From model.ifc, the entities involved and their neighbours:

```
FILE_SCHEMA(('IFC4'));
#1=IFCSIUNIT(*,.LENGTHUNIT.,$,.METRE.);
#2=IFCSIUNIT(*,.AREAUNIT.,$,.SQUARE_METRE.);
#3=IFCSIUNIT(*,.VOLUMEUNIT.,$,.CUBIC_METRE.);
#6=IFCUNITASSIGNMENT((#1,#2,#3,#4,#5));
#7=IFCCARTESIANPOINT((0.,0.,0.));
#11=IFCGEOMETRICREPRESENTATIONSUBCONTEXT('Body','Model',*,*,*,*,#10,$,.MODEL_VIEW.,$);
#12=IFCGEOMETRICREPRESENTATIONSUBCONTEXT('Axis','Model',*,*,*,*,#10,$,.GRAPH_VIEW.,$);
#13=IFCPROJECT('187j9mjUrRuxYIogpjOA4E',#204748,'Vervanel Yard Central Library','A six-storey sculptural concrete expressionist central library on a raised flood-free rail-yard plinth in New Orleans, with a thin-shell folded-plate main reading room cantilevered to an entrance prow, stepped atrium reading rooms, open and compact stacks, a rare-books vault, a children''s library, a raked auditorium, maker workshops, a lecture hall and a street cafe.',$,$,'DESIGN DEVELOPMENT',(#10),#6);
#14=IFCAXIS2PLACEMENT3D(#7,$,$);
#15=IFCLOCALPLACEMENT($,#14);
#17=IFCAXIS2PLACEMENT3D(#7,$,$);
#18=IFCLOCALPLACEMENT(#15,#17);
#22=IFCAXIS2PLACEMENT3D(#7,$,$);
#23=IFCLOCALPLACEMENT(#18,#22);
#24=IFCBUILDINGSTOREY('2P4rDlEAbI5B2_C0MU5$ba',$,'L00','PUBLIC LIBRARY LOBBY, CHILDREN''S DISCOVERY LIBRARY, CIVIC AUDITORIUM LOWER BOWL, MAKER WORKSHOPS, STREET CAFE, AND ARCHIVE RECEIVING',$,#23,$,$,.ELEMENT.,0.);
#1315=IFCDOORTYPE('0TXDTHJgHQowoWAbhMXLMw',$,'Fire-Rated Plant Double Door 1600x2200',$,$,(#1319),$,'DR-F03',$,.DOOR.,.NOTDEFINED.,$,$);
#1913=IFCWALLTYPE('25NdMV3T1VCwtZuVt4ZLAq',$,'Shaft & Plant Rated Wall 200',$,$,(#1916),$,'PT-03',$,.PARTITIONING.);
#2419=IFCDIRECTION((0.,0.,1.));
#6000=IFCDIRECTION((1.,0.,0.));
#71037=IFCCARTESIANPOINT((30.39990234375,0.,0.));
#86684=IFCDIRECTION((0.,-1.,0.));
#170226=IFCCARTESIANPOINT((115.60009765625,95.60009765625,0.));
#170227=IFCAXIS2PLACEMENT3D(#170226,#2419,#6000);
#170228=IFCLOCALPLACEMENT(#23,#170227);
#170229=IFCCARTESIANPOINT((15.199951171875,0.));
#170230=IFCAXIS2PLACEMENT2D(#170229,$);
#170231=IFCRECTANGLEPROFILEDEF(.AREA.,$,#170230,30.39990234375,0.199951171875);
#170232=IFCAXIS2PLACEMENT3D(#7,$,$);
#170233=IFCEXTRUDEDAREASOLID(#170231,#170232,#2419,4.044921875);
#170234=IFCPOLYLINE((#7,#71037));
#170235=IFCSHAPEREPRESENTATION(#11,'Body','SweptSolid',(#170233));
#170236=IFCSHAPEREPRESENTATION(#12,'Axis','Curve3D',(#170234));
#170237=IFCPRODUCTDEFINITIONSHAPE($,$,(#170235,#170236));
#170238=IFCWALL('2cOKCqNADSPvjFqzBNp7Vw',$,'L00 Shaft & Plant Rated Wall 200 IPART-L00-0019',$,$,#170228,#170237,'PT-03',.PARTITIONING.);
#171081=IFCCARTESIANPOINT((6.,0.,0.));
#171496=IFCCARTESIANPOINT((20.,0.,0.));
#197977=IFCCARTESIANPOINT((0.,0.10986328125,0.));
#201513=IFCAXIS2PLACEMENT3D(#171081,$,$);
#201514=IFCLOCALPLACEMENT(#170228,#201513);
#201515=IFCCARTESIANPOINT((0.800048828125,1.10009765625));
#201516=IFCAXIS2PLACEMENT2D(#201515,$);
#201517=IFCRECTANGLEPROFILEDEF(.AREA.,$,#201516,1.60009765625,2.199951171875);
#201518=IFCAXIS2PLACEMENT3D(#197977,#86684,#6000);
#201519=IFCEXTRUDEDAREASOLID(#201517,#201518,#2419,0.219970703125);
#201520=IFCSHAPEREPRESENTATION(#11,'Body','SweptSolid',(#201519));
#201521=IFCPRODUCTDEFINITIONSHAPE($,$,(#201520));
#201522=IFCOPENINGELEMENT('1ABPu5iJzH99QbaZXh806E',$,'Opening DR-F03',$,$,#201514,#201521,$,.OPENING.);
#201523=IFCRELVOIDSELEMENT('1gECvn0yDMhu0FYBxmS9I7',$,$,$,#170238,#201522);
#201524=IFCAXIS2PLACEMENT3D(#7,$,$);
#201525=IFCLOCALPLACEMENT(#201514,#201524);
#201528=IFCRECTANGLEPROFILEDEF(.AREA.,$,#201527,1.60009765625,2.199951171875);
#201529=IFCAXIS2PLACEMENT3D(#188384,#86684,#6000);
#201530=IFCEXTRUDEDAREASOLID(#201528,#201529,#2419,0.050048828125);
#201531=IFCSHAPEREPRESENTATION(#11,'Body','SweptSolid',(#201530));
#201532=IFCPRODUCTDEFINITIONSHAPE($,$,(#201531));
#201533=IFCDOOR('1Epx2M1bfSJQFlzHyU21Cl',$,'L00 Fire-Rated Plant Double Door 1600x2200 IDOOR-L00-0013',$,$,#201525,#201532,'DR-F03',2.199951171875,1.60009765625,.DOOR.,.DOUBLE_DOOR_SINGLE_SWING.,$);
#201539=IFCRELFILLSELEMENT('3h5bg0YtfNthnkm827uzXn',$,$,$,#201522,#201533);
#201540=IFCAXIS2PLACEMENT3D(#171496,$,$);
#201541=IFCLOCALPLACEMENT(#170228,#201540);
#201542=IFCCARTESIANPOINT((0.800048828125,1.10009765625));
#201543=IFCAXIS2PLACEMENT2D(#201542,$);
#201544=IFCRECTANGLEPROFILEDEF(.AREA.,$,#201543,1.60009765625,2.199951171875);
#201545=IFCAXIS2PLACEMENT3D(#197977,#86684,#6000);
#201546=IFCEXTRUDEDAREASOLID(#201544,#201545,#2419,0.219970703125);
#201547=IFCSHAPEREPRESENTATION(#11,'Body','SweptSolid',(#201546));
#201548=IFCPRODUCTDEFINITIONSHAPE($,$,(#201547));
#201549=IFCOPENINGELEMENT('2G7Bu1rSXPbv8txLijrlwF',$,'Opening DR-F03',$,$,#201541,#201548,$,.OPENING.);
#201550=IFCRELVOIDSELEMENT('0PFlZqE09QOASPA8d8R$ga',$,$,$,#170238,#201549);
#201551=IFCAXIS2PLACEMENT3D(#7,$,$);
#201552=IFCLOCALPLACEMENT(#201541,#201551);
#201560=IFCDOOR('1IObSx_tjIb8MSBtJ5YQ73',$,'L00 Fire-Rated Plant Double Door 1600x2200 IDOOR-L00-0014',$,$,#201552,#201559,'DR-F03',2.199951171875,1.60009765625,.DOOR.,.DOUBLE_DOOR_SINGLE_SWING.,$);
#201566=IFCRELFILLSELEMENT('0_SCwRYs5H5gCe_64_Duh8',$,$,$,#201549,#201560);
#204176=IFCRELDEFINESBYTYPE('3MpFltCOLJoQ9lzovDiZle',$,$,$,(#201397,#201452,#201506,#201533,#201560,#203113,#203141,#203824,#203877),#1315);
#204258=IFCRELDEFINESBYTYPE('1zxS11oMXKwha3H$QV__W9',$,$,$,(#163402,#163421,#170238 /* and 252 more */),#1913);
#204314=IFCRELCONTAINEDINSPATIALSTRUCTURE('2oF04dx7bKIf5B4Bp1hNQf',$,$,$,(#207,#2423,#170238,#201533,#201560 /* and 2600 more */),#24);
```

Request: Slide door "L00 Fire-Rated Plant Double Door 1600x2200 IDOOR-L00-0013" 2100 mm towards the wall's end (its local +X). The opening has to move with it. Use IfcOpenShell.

```python
import ifcopenshell
import ifcopenshell.api.geometry
import ifcopenshell.util.placement

model = ifcopenshell.open("model.ifc")

door = model.by_id(201533)
opening = door.FillsVoids[0].RelatingOpeningElement
wall = opening.VoidsElements[0].RelatingBuildingElement

wall_matrix = ifcopenshell.util.placement.get_local_placement(wall.ObjectPlacement)
shift = wall_matrix[:3, 0] * 2.1
before = ifcopenshell.util.placement.get_local_placement(door.ObjectPlacement)[:3, 3].copy()

# The door is placed relative to its opening, so it follows when the opening moves.
matrix = ifcopenshell.util.placement.get_local_placement(opening.ObjectPlacement)
matrix[:3, 3] += shift
ifcopenshell.api.geometry.edit_object_placement(
    model, product=opening, matrix=matrix, is_si=False, should_transform_children=True
)

after = ifcopenshell.util.placement.get_local_placement(door.ObjectPlacement)[:3, 3]
print("door moved by", (after - before).round(3) + 0.0)

model.write("model_updated.ifc")
```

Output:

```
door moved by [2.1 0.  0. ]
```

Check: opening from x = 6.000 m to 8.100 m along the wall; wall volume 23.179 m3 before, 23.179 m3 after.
